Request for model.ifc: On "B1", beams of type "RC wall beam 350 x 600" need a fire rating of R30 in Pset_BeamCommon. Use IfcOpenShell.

First a look at what the model holds.

```python
import ifcopenshell
import ifcopenshell.util.element

model = ifcopenshell.open("model.ifc")
print(model.schema)
storey = next(s for s in model.by_type("IfcBuildingStorey") if s.Name == "B1")
beams = [e for e in ifcopenshell.util.element.get_decomposition(storey) if e.is_a("IfcBeam")]
seen = {}
for e in beams:
    element_type = ifcopenshell.util.element.get_type(e)
    key = (element_type.Name if element_type != e and element_type else None, ifcopenshell.util.element.get_pset(e, "Pset_BeamCommon", "FireRating"))
    seen[key] = seen.get(key, 0) + 1
for (name, value), count in sorted(seen.items(), key=str):
    print(count, "x", name, "|", value)
```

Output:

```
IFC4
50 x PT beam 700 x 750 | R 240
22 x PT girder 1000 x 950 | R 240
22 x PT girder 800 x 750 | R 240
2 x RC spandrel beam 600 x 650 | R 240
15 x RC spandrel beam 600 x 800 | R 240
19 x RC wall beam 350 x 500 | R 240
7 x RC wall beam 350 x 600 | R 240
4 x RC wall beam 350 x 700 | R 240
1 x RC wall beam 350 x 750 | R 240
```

```python
import ifcopenshell
import ifcopenshell.api.pset
import ifcopenshell.util.element

model = ifcopenshell.open("model.ifc")

storey = next(s for s in model.by_type("IfcBuildingStorey") if s.Name == "B1")
beams = [e for e in ifcopenshell.util.element.get_decomposition(storey) if e.is_a("IfcBeam")]

count = 0
for e in beams:
    element_type = ifcopenshell.util.element.get_type(e)
    if element_type in (None, e) or element_type.Name != "RC wall beam 350 x 600":
        continue
    # add_pset returns the element's existing set when there is one.
    pset = ifcopenshell.api.pset.add_pset(model, product=e, name="Pset_BeamCommon")
    ifcopenshell.api.pset.edit_pset(model, pset=pset, properties={"FireRating": "R30"})
    count += 1

print(count, "beams updated")

model.write("model_rev.ifc")
```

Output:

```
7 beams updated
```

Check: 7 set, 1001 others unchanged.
